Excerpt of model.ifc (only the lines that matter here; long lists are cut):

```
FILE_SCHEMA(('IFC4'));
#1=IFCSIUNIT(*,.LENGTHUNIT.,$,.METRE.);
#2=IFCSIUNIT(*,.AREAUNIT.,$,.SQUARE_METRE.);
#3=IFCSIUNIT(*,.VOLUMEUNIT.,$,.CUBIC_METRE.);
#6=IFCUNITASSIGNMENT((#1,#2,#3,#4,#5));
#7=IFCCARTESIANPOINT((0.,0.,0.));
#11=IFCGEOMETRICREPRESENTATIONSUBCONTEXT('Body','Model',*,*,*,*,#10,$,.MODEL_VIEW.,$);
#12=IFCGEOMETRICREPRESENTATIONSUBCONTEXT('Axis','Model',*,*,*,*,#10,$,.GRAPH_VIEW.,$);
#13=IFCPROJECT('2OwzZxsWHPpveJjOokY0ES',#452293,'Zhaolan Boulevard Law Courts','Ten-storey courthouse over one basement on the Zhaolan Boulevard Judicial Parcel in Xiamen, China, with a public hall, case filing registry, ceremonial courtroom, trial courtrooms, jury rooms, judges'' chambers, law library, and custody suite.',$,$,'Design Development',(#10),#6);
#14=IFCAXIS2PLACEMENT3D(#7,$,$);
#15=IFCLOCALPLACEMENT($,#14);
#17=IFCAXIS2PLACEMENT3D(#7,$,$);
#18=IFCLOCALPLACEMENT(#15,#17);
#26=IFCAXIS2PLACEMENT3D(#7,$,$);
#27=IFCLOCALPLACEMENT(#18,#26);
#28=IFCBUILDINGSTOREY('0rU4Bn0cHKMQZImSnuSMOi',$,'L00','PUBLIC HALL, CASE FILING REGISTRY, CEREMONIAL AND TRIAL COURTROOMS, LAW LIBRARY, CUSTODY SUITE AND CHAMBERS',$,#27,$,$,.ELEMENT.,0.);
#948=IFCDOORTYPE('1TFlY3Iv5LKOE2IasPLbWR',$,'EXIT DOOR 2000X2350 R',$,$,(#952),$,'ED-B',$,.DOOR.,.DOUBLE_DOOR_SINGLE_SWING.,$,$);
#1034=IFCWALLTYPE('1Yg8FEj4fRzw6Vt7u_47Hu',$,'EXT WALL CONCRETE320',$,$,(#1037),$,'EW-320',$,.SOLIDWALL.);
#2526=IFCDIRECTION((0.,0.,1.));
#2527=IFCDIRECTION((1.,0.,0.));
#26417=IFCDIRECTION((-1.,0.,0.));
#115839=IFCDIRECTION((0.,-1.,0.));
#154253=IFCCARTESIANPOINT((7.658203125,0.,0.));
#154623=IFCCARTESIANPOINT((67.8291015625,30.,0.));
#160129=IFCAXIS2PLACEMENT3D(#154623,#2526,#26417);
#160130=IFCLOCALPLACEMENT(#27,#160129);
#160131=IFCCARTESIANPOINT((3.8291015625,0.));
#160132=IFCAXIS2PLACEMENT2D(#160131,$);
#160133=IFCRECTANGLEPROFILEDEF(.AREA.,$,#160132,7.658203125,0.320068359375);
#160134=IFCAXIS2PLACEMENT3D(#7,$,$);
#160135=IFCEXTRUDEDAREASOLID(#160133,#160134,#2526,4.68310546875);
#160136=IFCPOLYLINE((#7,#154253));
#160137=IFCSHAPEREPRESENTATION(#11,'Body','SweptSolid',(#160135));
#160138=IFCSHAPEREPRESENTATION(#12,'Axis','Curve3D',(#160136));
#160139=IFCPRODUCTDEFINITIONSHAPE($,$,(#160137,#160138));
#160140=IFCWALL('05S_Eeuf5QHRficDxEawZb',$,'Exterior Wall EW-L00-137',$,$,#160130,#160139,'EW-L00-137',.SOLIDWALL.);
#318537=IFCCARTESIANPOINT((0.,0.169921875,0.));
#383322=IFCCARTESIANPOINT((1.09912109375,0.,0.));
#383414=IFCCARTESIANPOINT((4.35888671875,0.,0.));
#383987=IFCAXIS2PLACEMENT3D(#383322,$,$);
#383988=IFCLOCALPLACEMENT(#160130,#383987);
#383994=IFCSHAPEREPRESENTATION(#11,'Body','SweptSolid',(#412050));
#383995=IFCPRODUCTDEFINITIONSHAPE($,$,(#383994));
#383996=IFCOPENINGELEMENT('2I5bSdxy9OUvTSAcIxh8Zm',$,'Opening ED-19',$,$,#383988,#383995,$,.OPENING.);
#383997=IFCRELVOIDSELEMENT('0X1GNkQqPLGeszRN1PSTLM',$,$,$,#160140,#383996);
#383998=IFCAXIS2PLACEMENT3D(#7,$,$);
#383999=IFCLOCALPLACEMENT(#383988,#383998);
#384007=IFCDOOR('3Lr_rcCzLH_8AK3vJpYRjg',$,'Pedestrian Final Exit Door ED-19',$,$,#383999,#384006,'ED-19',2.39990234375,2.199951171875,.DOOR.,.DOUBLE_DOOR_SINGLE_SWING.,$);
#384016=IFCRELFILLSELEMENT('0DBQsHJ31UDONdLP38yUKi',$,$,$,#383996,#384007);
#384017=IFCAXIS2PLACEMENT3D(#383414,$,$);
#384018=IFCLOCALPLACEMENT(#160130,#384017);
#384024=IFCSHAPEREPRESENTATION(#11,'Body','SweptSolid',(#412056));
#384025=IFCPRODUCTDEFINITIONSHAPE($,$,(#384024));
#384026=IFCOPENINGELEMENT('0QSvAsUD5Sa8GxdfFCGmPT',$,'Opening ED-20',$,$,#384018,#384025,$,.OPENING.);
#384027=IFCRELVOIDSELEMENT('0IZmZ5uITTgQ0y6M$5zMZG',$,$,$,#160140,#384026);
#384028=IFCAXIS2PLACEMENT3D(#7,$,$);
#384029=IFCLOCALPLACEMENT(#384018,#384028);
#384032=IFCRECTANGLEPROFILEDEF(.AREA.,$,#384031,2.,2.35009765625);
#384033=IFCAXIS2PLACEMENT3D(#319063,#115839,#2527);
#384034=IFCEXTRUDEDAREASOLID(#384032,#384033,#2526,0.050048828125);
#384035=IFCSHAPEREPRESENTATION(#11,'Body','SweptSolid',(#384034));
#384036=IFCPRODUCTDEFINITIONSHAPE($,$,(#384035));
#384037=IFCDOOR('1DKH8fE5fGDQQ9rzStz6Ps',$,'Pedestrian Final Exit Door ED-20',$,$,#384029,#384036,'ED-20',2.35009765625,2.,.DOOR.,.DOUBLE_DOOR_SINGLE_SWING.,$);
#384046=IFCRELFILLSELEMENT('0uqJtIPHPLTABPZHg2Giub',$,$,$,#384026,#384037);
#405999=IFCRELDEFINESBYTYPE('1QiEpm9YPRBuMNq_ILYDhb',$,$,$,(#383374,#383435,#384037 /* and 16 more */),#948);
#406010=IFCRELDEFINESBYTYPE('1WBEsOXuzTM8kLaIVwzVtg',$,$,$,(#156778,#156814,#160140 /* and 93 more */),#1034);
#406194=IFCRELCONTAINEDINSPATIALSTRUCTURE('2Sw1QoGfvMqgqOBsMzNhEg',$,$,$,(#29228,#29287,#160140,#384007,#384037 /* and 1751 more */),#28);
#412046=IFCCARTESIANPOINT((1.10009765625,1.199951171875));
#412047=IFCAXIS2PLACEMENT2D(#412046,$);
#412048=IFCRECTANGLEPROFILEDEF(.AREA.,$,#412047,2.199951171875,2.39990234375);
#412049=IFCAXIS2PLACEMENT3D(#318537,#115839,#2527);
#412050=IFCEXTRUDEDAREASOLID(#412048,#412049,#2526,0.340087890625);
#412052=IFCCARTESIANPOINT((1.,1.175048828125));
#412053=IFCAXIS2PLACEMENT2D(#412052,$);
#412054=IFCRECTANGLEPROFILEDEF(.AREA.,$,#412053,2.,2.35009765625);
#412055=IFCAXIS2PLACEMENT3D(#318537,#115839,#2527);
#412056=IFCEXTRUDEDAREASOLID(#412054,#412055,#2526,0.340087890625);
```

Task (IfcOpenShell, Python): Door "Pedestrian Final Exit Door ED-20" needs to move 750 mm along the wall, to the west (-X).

```python
import ifcopenshell
import ifcopenshell.api.geometry
import ifcopenshell.util.placement

model = ifcopenshell.open("model.ifc")

door = model.by_id(384037)
opening = door.FillsVoids[0].RelatingOpeningElement
wall = opening.VoidsElements[0].RelatingBuildingElement

wall_matrix = ifcopenshell.util.placement.get_local_placement(wall.ObjectPlacement)
shift = wall_matrix[:3, 0] * 0.75
before = ifcopenshell.util.placement.get_local_placement(door.ObjectPlacement)[:3, 3].copy()

# The door is placed relative to its opening, so it follows when the opening moves.
matrix = ifcopenshell.util.placement.get_local_placement(opening.ObjectPlacement)
matrix[:3, 3] += shift
ifcopenshell.api.geometry.edit_object_placement(
    model, product=opening, matrix=matrix, is_si=False, should_transform_children=True
)

after = ifcopenshell.util.placement.get_local_placement(door.ObjectPlacement)[:3, 3]
print("door moved by", (after - before).round(3) + 0.0)

model.write("model_rev.ifc")
```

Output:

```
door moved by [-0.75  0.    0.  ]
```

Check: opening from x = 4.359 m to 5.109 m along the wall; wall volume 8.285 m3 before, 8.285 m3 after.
